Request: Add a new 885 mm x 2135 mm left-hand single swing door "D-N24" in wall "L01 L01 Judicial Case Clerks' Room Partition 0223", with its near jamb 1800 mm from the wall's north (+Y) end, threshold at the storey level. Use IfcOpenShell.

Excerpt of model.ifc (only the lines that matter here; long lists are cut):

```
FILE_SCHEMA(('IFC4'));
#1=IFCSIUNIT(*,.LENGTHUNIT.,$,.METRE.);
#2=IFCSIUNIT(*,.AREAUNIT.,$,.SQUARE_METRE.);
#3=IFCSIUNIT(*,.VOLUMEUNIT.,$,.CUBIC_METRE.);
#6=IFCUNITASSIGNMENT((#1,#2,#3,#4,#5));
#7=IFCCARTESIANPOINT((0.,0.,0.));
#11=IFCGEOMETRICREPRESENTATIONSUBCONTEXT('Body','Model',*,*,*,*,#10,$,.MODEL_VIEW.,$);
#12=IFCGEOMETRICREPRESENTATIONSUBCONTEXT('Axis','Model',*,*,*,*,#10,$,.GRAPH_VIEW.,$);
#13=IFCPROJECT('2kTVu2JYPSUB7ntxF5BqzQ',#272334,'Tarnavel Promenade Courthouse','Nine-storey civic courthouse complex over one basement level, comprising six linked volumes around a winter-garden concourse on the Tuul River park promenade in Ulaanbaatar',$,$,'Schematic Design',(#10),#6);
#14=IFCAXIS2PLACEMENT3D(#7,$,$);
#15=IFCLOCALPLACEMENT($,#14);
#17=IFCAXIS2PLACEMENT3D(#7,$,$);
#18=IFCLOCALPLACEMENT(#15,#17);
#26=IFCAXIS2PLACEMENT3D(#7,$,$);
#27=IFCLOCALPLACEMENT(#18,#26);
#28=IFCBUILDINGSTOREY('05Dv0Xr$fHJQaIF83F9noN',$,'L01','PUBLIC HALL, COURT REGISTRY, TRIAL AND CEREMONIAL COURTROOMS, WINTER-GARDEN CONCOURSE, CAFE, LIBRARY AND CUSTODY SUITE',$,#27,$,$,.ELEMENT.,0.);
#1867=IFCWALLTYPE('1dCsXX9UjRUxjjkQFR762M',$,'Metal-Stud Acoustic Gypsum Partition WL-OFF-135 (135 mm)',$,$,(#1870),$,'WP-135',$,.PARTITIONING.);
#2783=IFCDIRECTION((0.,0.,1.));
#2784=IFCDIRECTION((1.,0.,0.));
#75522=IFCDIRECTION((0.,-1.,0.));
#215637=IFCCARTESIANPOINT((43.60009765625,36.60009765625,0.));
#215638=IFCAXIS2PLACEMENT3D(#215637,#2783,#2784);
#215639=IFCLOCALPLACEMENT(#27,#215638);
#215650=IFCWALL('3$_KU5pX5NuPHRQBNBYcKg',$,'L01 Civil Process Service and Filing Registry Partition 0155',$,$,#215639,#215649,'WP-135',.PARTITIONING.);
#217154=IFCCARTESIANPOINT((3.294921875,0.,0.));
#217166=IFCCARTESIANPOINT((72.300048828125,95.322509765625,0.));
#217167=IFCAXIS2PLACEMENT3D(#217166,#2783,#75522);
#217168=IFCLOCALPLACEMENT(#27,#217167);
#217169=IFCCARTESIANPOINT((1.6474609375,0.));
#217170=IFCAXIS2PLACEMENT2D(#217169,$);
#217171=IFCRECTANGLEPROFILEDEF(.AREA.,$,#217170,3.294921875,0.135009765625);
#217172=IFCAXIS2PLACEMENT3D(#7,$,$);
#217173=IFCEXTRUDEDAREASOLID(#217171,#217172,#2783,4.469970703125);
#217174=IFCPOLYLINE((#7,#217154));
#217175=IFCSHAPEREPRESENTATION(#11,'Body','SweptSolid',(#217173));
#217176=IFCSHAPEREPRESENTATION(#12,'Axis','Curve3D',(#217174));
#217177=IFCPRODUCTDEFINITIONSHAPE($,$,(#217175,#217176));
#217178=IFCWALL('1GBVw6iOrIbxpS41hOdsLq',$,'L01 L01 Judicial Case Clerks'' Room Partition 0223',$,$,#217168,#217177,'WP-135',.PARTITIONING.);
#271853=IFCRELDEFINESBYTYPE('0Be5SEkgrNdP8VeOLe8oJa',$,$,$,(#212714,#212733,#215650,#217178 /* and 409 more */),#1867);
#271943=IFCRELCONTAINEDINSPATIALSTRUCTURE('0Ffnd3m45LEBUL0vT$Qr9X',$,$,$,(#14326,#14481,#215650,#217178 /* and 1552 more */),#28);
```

```python
import numpy as np
import ifcopenshell
import ifcopenshell.api.feature
import ifcopenshell.api.geometry
import ifcopenshell.api.root
import ifcopenshell.api.spatial
import ifcopenshell.geom
import ifcopenshell.util.element
import ifcopenshell.util.placement
import ifcopenshell.util.representation
import ifcopenshell.util.shape
import ifcopenshell.util.unit

model = ifcopenshell.open("model.ifc")
unit_scale = ifcopenshell.util.unit.calculate_unit_scale(model)
settings = ifcopenshell.geom.settings()


def volume(element):
    """Net volume in cubic metres, openings subtracted."""
    shape = ifcopenshell.geom.create_shape(settings, element)
    return ifcopenshell.util.shape.get_volume(shape.geometry)


wall = model.by_guid("1GBVw6iOrIbxpS41hOdsLq")
storey = ifcopenshell.util.element.get_container(wall, ifc_class="IfcBuildingStorey")
context = ifcopenshell.util.representation.get_context(model, "Model", "Body", "MODEL_VIEW")
before = volume(wall)

width, height, from_end, sill = 0.885, 2.135, 1.8, 0.0  # metres

# The wall runs along its own X axis, and the end named is its -X end.
wall_shape = ifcopenshell.geom.create_shape(settings, wall)
x, y, z = ifcopenshell.util.shape.get_vertices(wall_shape.geometry).T
start = x.min() + from_end
face, thickness = float(y.min()), float(y.max() - y.min())
wall_matrix = ifcopenshell.util.placement.get_local_placement(wall.ObjectPlacement)
level = ifcopenshell.util.placement.get_local_placement(storey.ObjectPlacement)[2, 3]


def in_wall(x, y):
    """Placement at x, y metres in the wall's axes, at sill height."""
    matrix = wall_matrix.copy()
    matrix[:, 3] = wall_matrix @ np.array([x / unit_scale, y / unit_scale, 0.0, 1.0])
    matrix[2, 3] = level + sill / unit_scale
    return matrix


# Opening: a box that overshoots both wall faces by 50 mm.
opening = ifcopenshell.api.root.create_entity(model, ifc_class="IfcOpeningElement", predefined_type="OPENING")
box = ifcopenshell.api.geometry.add_wall_representation(
    model, context=context, length=width, height=height, thickness=thickness + 0.1
)
ifcopenshell.api.geometry.assign_representation(model, product=opening, representation=box)
ifcopenshell.api.geometry.edit_object_placement(model, product=opening, matrix=in_wall(start, face - 0.05), is_si=False)
ifcopenshell.api.feature.add_feature(model, feature=opening, element=wall)

door = ifcopenshell.api.root.create_entity(model, ifc_class="IfcDoor", name="D-N24", predefined_type="DOOR")
door.OverallWidth, door.OverallHeight = width / unit_scale, height / unit_scale
door.OperationType = "SINGLE_SWING_LEFT"
body = ifcopenshell.api.geometry.add_door_representation(
    model,
    context=context,
    overall_width=door.OverallWidth,
    overall_height=door.OverallHeight,
    operation_type="SINGLE_SWING_LEFT",
    lining_properties={"LiningDepth": thickness / unit_scale, "ThresholdDepth": thickness / unit_scale},
)
ifcopenshell.api.geometry.assign_representation(model, product=door, representation=body)
ifcopenshell.api.spatial.assign_container(model, products=[door], relating_structure=storey)
ifcopenshell.api.feature.add_filling(model, opening=opening, element=door)

# The lining spans the wall, so the door starts at the wall face.
ifcopenshell.api.geometry.edit_object_placement(model, product=door, matrix=in_wall(start, face), is_si=False)

after = volume(wall)

print(f"wall volume {before:.3f} -> {after:.3f} m3")

model.write("model_v2.ifc")
```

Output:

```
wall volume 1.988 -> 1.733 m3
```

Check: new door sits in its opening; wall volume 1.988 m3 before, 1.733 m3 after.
